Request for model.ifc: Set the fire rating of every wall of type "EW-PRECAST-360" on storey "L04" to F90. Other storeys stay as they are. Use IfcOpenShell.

First a look at what the model holds.

```python
import ifcopenshell
import ifcopenshell.util.element

model = ifcopenshell.open("model.ifc")
print(model.schema)
storey = next(s for s in model.by_type("IfcBuildingStorey") if s.Name == "L04")
walls = [e for e in ifcopenshell.util.element.get_decomposition(storey) if e.is_a("IfcWall")]
seen = {}
for e in walls:
    element_type = ifcopenshell.util.element.get_type(e)
    key = (element_type.Name if element_type != e and element_type else None, ifcopenshell.util.element.get_pset(e, "Pset_WallCommon", "FireRating"))
    seen[key] = seen.get(key, 0) + 1
for (name, value), count in sorted(seen.items(), key=str):
    print(count, "x", name, "|", value)
```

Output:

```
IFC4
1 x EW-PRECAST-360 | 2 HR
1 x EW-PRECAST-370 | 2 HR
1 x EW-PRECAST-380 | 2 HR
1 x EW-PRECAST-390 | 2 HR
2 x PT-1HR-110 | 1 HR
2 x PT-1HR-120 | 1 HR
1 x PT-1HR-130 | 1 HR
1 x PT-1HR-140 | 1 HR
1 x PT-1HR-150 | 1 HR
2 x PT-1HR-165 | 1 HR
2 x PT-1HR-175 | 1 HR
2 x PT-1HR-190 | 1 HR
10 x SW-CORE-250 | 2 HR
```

```python
import ifcopenshell
import ifcopenshell.api.pset
import ifcopenshell.util.element

model = ifcopenshell.open("model.ifc")

storey = next(s for s in model.by_type("IfcBuildingStorey") if s.Name == "L04")
walls = [e for e in ifcopenshell.util.element.get_decomposition(storey) if e.is_a("IfcWall")]

count = 0
for e in walls:
    element_type = ifcopenshell.util.element.get_type(e)
    if element_type in (None, e) or element_type.Name != "EW-PRECAST-360":
        continue
    # add_pset returns the element's existing set when there is one.
    pset = ifcopenshell.api.pset.add_pset(model, product=e, name="Pset_WallCommon")
    ifcopenshell.api.pset.edit_pset(model, pset=pset, properties={"FireRating": "F90"})
    count += 1

print(count, "walls updated")

model.write("model_updated.ifc")
```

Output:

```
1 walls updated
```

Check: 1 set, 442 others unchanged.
